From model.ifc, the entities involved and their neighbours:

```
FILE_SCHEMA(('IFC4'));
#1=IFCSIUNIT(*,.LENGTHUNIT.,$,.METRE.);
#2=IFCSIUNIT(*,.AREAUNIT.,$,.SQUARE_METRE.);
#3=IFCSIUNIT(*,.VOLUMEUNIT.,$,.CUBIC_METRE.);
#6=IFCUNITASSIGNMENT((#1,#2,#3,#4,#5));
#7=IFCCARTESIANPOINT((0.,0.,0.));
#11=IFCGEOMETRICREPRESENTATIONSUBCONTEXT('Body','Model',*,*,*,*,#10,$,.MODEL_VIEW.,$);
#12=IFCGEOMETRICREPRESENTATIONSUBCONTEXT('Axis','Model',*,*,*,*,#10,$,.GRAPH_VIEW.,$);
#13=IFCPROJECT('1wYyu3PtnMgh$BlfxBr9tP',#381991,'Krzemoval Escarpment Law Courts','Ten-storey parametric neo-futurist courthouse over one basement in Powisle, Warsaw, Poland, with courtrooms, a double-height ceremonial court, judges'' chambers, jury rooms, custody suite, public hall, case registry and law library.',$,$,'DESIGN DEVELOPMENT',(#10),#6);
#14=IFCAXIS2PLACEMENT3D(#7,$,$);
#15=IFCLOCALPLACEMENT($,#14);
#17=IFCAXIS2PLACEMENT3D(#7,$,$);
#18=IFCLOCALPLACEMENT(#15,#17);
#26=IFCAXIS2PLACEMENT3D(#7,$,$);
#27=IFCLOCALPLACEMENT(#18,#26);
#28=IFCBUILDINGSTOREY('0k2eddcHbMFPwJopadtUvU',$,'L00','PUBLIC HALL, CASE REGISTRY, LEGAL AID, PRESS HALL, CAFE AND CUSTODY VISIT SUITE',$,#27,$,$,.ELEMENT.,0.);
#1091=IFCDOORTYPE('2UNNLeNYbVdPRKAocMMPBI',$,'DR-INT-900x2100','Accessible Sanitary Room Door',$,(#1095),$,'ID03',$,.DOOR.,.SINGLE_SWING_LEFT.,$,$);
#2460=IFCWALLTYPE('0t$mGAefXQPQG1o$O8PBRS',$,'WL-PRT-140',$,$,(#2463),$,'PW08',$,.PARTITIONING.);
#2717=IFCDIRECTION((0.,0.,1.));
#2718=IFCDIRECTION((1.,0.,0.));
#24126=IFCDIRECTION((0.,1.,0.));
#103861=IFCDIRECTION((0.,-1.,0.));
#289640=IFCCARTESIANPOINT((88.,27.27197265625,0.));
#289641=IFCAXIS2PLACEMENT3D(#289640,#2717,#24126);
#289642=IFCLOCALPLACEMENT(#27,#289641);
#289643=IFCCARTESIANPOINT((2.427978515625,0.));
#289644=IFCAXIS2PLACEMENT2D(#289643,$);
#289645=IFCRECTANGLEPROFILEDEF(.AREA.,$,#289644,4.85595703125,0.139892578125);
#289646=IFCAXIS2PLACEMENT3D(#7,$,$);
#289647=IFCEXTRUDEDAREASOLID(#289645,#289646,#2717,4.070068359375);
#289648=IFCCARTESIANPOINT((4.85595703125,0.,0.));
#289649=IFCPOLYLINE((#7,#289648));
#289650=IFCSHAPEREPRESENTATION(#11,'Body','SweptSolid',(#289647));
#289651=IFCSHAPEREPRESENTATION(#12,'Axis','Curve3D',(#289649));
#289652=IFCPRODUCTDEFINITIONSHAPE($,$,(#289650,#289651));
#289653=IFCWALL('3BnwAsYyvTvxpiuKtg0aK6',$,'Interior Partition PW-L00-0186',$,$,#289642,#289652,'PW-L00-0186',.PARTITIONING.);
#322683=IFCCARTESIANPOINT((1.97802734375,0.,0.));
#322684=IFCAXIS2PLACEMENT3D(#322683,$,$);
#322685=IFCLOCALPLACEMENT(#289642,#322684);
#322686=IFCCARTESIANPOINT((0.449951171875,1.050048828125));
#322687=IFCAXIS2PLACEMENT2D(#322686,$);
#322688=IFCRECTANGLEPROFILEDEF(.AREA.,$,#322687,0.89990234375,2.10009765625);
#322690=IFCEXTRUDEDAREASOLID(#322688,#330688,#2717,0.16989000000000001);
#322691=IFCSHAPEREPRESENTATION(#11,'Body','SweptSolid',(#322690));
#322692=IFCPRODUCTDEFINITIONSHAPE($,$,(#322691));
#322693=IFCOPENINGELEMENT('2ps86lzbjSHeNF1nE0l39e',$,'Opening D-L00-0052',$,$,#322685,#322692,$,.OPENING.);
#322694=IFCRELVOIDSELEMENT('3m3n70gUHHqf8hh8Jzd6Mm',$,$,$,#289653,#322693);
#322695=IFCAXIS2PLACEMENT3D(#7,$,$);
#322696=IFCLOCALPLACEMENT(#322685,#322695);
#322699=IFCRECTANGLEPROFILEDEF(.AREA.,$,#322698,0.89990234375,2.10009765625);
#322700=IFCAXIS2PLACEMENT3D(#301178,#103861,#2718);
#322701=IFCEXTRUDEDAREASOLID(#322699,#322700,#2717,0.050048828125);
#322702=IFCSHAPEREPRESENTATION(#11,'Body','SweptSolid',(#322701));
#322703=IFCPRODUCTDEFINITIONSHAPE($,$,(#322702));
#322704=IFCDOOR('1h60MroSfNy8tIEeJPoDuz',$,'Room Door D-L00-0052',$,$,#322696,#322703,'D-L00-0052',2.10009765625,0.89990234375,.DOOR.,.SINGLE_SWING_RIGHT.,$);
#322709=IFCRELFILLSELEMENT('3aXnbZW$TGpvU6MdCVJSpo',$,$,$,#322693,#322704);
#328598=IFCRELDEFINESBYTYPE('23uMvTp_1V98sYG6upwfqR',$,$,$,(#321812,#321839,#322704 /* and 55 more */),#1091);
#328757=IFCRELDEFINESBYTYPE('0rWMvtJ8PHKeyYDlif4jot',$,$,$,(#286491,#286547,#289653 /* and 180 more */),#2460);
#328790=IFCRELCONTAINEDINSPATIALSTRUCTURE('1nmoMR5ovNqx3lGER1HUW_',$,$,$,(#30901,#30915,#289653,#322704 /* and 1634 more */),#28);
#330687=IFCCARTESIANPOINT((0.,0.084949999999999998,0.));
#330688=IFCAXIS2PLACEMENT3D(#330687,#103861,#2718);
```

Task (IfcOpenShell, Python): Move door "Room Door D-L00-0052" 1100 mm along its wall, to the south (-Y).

```python
import ifcopenshell
import ifcopenshell.api.geometry
import ifcopenshell.util.placement

model = ifcopenshell.open("model.ifc")

door = model.by_guid("1h60MroSfNy8tIEeJPoDuz")
opening = door.FillsVoids[0].RelatingOpeningElement
wall = opening.VoidsElements[0].RelatingBuildingElement

wall_matrix = ifcopenshell.util.placement.get_local_placement(wall.ObjectPlacement)
shift = wall_matrix[:3, 0] * -1.1
before = ifcopenshell.util.placement.get_local_placement(door.ObjectPlacement)[:3, 3].copy()

# The door is placed relative to its opening, so it follows when the opening moves.
matrix = ifcopenshell.util.placement.get_local_placement(opening.ObjectPlacement)
matrix[:3, 3] += shift
ifcopenshell.api.geometry.edit_object_placement(
    model, product=opening, matrix=matrix, is_si=False, should_transform_children=True
)

after = ifcopenshell.util.placement.get_local_placement(door.ObjectPlacement)[:3, 3]
print("door moved by", (after - before).round(3) + 0.0)

model.write("model_rev.ifc")
```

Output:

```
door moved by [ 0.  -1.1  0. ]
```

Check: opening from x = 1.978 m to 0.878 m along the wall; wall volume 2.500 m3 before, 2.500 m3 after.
